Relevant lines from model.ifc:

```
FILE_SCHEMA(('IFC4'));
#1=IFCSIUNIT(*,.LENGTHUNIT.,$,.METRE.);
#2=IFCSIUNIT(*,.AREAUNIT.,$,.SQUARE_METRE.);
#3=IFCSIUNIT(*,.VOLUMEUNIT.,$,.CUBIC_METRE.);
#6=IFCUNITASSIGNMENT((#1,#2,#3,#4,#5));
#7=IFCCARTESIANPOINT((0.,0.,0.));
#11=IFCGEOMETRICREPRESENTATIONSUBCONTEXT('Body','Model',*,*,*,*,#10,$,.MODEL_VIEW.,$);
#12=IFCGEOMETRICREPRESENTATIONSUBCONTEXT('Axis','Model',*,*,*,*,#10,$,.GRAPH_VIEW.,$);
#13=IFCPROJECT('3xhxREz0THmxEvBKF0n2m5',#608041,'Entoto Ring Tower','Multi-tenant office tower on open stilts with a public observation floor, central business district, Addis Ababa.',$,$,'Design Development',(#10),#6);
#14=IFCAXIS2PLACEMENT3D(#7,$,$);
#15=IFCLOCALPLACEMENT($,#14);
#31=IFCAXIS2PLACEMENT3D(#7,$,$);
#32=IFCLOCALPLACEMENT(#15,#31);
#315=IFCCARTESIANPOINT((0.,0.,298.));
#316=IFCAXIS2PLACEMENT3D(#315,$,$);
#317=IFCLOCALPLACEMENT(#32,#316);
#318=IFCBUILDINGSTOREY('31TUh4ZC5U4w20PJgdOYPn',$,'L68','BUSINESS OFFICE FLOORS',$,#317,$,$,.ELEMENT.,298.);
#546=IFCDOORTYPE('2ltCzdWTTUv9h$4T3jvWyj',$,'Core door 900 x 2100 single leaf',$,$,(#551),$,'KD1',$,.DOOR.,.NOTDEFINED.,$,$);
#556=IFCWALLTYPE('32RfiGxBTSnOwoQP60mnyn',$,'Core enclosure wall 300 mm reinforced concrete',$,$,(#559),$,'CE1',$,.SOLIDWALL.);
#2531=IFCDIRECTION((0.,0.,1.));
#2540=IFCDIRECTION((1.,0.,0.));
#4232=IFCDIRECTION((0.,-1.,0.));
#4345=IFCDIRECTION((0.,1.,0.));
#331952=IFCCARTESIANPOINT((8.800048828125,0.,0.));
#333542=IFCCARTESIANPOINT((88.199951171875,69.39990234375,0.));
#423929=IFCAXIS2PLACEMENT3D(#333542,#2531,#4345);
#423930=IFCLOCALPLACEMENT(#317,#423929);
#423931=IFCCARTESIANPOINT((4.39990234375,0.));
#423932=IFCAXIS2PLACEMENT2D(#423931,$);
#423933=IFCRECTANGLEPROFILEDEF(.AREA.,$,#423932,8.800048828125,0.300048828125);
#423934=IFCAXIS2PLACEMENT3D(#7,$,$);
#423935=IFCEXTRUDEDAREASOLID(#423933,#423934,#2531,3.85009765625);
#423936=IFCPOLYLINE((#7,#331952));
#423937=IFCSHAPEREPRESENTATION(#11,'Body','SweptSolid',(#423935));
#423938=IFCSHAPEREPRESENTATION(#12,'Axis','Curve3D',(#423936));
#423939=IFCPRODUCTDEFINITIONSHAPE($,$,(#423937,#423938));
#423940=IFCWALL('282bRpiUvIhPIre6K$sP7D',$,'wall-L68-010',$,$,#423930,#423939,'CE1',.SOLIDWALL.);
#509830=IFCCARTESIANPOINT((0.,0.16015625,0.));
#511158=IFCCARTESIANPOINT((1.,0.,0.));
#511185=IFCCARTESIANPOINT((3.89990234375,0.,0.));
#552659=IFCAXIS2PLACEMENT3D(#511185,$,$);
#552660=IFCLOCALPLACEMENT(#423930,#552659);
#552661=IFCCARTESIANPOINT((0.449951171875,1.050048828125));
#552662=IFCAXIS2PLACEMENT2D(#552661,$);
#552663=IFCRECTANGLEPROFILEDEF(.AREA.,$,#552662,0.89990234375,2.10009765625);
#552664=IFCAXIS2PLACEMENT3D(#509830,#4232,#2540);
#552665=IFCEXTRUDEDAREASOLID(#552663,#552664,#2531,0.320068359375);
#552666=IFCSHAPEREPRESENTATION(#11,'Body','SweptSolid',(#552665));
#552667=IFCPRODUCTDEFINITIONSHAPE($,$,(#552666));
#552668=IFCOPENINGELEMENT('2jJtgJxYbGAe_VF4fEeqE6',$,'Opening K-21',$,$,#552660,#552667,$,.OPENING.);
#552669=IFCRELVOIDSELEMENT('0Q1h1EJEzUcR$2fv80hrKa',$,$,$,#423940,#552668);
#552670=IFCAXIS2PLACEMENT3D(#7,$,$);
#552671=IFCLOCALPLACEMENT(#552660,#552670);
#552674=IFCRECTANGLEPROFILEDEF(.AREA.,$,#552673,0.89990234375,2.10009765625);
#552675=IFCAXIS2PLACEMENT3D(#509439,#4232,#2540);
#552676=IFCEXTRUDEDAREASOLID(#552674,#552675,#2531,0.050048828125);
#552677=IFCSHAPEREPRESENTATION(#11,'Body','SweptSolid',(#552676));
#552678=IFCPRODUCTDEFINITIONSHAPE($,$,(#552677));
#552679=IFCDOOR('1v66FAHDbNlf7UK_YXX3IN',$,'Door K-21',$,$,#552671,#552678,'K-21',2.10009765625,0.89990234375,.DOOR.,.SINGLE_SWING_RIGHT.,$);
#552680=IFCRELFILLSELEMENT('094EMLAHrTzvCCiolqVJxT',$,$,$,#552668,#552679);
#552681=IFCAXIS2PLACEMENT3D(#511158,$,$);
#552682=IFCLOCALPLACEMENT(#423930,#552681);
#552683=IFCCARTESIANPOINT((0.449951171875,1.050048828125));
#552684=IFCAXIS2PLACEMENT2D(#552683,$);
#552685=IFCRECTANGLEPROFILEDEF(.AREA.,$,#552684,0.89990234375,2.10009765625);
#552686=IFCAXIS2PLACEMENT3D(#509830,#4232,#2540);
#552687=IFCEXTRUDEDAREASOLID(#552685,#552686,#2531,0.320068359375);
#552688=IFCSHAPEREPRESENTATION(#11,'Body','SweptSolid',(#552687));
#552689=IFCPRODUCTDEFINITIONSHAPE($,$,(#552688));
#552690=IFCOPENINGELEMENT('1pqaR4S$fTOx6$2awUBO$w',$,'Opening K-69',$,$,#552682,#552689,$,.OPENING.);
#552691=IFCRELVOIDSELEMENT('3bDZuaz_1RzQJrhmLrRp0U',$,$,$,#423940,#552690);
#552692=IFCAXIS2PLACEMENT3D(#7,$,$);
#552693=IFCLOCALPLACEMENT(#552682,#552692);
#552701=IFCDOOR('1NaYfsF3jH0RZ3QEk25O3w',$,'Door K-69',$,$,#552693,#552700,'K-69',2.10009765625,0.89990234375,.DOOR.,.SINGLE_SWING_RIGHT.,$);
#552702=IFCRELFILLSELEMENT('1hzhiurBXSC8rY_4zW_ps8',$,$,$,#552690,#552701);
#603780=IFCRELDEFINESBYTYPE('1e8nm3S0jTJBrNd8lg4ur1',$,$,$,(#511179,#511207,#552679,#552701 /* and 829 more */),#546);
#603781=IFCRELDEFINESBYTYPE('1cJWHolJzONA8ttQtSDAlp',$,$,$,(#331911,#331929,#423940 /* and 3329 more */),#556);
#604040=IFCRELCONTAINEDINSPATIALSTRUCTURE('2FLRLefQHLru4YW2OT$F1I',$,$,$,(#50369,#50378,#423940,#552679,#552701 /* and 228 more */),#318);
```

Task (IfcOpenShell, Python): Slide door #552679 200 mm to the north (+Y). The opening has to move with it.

```python
import ifcopenshell
import ifcopenshell.api.geometry
import ifcopenshell.util.placement
import ifcopenshell.util.unit

model = ifcopenshell.open("model.ifc")
unit_scale = ifcopenshell.util.unit.calculate_unit_scale(model)

door = model.by_guid("1v66FAHDbNlf7UK_YXX3IN")
opening = door.FillsVoids[0].RelatingOpeningElement
wall = opening.VoidsElements[0].RelatingBuildingElement

wall_matrix = ifcopenshell.util.placement.get_local_placement(wall.ObjectPlacement)
shift = wall_matrix[:3, 0] * 0.2 / unit_scale
before = ifcopenshell.util.placement.get_local_placement(door.ObjectPlacement)[:3, 3].copy()

# The door is placed relative to its opening, so it follows when the opening moves.
matrix = ifcopenshell.util.placement.get_local_placement(opening.ObjectPlacement)
matrix[:3, 3] += shift
ifcopenshell.api.geometry.edit_object_placement(
    model, product=opening, matrix=matrix, is_si=False, should_transform_children=True
)

after = ifcopenshell.util.placement.get_local_placement(door.ObjectPlacement)[:3, 3]
print("door moved by", (after - before).round(3) + 0.0)

model.write("model_rev.ifc")
```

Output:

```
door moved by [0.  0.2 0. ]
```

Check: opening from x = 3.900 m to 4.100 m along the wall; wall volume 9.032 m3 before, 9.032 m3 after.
